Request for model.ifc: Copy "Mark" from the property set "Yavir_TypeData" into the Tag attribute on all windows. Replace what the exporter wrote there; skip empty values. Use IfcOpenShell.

First a look at what the model holds.

```python
import ifcopenshell
import ifcopenshell.util.element

model = ifcopenshell.open("model.ifc")
print(model.schema)
windows = model.by_type("IfcWindow")
print(len(windows), "windows")
for e in windows[:8]:
    source = ifcopenshell.util.element.get_pset(e, "Yavir_TypeData", "Mark")
    target = e.Tag
    print(e.id(), repr(source), repr(target), sep=" | ")
```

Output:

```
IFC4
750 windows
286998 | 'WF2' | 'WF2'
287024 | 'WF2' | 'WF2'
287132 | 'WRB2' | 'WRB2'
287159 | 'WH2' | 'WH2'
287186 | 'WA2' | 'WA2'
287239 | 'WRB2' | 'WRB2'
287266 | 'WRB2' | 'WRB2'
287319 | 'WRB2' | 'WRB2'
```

```python
import ifcopenshell
import ifcopenshell.util.element

model = ifcopenshell.open("model.ifc")

count = 0
for e in model.by_type("IfcWindow"):
    value = ifcopenshell.util.element.get_pset(e, "Yavir_TypeData", "Mark")
    current = e.Tag
    if not value or not value.strip() or current == value:
        continue
    e.Tag = value
    count += 1

print(count, "windows updated")

model.write("model_rev.ifc")
```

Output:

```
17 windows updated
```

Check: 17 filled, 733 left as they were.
